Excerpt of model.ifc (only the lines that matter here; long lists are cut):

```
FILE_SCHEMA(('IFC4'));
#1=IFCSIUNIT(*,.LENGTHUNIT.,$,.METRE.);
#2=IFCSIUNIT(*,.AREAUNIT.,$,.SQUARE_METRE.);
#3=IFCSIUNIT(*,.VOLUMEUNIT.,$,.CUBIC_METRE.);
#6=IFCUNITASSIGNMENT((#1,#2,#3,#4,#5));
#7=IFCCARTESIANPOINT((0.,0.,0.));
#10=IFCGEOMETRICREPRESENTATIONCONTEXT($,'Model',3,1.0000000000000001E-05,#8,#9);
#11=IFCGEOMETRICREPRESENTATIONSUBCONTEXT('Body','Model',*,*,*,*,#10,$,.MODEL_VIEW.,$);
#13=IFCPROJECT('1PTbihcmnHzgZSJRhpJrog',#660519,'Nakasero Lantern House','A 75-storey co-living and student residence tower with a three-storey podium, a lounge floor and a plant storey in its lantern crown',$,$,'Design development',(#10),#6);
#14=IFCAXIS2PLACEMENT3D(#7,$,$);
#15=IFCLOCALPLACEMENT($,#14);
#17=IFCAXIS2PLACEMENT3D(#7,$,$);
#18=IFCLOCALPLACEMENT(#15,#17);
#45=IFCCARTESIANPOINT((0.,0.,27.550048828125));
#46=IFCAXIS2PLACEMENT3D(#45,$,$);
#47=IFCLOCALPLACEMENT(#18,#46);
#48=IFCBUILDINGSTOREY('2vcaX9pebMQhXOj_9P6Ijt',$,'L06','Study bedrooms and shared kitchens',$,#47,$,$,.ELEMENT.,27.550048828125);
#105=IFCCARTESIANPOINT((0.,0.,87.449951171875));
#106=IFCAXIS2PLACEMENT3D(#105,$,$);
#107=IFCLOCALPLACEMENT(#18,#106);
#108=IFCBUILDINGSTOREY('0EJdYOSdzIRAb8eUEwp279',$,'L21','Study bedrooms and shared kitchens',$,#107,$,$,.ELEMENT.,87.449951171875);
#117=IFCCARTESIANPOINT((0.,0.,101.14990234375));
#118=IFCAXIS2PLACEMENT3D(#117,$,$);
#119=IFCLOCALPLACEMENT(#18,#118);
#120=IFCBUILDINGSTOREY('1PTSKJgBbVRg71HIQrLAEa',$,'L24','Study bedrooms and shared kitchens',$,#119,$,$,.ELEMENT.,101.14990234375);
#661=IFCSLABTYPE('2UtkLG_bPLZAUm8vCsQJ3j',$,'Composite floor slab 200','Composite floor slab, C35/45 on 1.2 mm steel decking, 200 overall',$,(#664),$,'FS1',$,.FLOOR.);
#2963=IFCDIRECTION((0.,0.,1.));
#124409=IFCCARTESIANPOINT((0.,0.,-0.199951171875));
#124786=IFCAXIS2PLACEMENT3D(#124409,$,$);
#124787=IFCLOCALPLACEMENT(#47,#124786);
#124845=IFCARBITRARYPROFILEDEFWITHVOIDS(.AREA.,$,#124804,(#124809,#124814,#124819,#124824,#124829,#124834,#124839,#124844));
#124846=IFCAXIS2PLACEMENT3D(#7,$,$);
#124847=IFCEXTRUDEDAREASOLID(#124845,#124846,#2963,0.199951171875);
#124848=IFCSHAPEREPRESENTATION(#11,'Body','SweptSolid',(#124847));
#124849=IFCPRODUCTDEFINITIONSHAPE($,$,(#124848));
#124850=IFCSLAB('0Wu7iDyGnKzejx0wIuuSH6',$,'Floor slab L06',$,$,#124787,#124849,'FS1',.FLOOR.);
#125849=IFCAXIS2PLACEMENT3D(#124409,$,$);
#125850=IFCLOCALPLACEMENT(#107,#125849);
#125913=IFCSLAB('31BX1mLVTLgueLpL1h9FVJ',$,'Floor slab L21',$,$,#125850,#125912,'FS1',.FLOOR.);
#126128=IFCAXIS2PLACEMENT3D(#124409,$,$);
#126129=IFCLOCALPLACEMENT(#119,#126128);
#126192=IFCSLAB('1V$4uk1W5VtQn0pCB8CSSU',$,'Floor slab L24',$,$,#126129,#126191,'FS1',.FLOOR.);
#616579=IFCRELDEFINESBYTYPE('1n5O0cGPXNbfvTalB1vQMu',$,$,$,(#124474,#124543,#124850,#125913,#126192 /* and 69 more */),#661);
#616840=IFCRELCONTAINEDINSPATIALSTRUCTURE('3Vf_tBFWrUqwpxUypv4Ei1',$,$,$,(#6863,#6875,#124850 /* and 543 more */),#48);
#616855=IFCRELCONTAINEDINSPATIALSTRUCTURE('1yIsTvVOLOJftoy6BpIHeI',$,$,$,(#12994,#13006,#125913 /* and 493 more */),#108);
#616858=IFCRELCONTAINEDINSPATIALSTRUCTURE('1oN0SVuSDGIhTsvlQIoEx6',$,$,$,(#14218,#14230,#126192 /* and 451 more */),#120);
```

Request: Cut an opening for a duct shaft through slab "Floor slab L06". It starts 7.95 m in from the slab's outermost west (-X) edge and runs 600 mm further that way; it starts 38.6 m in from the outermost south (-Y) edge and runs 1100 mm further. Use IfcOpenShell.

```python
import numpy as np
import ifcopenshell
import ifcopenshell.api.feature
import ifcopenshell.api.geometry
import ifcopenshell.api.root
import ifcopenshell.geom
import ifcopenshell.util.placement
import ifcopenshell.util.representation
import ifcopenshell.util.shape
import ifcopenshell.util.unit

model = ifcopenshell.open("model.ifc")
unit_scale = ifcopenshell.util.unit.calculate_unit_scale(model)
settings = ifcopenshell.geom.settings()


def volume(element):
    """Net volume in cubic metres, openings subtracted."""
    shape = ifcopenshell.geom.create_shape(settings, element)
    return ifcopenshell.util.shape.get_volume(shape.geometry)


slab = model.by_guid("0Wu7iDyGnKzejx0wIuuSH6")
before = volume(slab)

# Extent in the slab's own axes, in metres. The edges named are its -X and -Y sides.
slab_shape = ifcopenshell.geom.create_shape(settings, slab)
vertices = ifcopenshell.util.shape.get_vertices(slab_shape.geometry)
x_min, y_min, bottom = vertices.min(axis=0)
top = vertices[:, 2].max()

opening = ifcopenshell.api.root.create_entity(model, ifc_class="IfcOpeningElement", name="Duct shaft opening", predefined_type="OPENING")
context = ifcopenshell.util.representation.get_context(model, "Model", "Body", "MODEL_VIEW")
width, depth = 0.6, 1.1
outline = [(0.0, 0.0), (width, 0.0), (width, depth), (0.0, depth), (0.0, 0.0)]
# Overshoot both faces by 50 mm so the cut is clean.
shape = ifcopenshell.api.geometry.add_slab_representation(
    model, context=context, depth=top - bottom + 0.1, polyline=outline
)
ifcopenshell.api.geometry.assign_representation(model, product=opening, representation=shape)

matrix = ifcopenshell.util.placement.get_local_placement(slab.ObjectPlacement)
matrix[:, 3] = matrix @ np.append(np.array([x_min + 7.95, y_min + 38.6, bottom - 0.05]) / unit_scale, 1.0)
ifcopenshell.api.geometry.edit_object_placement(model, product=opening, matrix=matrix, is_si=False)
ifcopenshell.api.feature.add_feature(model, feature=opening, element=slab)

after = volume(slab)

print(f"slab volume {before:.3f} -> {after:.3f} m3")

model.write("model_edited.ifc")
```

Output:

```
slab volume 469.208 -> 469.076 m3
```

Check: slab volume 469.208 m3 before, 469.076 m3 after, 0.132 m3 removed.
